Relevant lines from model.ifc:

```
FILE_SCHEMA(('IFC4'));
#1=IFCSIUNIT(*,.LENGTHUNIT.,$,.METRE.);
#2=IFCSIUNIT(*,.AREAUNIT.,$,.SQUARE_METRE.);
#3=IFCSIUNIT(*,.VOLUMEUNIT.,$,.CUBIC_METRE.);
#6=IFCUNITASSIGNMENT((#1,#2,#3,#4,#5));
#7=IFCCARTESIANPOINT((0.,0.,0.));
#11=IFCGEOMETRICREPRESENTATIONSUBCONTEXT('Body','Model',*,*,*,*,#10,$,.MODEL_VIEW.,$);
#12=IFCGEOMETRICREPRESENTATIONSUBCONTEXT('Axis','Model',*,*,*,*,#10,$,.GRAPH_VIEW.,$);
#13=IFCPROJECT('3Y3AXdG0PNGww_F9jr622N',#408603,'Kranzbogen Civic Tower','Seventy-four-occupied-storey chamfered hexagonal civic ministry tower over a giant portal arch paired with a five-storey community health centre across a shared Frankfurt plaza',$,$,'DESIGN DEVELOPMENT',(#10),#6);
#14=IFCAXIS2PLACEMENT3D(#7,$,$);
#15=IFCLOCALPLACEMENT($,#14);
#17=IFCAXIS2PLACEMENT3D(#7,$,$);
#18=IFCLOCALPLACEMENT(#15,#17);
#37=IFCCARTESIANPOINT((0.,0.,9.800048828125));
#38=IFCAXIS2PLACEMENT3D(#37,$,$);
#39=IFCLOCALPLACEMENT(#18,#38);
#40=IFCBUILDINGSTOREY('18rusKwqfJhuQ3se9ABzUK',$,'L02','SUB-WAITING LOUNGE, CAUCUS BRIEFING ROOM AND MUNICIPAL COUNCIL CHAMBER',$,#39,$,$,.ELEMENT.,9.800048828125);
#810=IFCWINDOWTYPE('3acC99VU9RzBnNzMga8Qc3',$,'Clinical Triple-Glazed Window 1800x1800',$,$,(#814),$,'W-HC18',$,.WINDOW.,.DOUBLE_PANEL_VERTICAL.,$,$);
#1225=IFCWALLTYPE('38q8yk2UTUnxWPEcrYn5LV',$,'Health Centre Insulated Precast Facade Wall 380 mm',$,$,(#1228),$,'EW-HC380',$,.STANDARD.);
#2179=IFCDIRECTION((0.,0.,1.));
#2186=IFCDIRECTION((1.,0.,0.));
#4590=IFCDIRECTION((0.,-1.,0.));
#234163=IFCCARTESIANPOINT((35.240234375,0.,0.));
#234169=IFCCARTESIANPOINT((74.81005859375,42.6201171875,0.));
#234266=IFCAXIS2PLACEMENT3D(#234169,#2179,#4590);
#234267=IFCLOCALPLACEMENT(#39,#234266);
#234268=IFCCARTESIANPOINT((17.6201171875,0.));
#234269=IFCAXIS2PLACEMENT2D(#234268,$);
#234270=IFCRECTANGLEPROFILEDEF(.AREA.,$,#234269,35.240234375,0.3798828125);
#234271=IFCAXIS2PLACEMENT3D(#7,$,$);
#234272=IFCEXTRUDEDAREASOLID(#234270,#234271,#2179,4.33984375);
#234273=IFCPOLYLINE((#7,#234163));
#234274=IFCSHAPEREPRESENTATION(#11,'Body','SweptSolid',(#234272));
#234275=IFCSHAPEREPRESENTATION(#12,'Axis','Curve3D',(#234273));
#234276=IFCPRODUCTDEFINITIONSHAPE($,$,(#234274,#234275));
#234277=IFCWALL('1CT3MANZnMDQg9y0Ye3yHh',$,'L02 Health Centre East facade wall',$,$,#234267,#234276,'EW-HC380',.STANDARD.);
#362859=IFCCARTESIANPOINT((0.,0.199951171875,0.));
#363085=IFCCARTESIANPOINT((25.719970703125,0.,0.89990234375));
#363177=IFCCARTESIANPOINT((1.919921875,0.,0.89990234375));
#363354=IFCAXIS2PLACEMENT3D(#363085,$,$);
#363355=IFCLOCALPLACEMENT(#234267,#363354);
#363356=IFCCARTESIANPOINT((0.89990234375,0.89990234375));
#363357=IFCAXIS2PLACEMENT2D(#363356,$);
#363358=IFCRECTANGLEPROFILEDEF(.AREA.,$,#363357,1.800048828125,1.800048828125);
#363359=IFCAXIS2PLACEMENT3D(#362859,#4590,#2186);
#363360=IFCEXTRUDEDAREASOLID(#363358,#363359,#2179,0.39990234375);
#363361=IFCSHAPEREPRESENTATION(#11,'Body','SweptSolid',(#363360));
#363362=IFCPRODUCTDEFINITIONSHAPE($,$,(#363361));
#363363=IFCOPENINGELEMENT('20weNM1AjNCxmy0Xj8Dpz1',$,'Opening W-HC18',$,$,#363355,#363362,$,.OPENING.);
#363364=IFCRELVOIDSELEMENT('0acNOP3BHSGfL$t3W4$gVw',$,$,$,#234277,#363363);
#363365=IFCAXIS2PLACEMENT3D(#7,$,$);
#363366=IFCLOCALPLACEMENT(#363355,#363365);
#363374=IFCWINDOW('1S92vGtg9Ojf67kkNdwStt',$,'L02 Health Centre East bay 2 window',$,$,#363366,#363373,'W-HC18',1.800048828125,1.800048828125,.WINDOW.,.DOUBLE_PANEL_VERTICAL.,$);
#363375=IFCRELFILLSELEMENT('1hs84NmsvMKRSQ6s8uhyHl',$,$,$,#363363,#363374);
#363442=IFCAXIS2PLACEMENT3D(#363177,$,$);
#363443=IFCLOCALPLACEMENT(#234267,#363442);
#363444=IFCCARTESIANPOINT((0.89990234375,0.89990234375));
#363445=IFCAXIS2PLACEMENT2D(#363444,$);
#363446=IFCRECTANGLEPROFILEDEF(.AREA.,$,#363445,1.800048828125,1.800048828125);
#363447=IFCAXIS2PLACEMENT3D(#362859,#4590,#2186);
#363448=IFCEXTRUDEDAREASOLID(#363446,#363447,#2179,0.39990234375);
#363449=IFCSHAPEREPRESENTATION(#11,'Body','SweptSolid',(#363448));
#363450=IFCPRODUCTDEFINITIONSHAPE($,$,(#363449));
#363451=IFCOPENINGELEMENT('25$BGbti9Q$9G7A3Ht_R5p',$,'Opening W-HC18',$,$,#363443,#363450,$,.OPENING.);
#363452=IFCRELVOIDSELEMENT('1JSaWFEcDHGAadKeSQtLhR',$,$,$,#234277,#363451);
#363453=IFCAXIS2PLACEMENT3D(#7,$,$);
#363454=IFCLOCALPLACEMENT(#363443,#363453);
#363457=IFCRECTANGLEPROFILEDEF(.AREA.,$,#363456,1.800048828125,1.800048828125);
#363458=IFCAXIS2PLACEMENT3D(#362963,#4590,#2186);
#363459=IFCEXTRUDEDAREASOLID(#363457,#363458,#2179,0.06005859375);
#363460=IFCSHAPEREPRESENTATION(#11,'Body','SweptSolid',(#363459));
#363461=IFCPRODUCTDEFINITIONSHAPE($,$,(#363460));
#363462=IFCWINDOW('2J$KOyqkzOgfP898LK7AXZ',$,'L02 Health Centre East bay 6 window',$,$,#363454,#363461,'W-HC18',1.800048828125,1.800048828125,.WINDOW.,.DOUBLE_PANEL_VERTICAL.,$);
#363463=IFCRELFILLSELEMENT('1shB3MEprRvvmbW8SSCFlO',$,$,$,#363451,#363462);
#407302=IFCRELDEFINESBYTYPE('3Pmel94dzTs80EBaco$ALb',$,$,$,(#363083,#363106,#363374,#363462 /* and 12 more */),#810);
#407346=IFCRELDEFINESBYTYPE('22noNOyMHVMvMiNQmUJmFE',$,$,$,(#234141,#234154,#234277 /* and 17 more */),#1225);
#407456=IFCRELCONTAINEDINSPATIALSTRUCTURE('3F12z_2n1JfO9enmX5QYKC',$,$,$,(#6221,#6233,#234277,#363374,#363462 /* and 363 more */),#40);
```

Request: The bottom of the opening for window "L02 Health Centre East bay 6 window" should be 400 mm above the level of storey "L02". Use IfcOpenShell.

```python
import numpy as np
import ifcopenshell
import ifcopenshell.api.geometry
import ifcopenshell.geom
import ifcopenshell.util.element
import ifcopenshell.util.placement
import ifcopenshell.util.shape
import ifcopenshell.util.unit

model = ifcopenshell.open("model.ifc")
unit_scale = ifcopenshell.util.unit.calculate_unit_scale(model)

window = model.by_id(363462)
opening = window.FillsVoids[0].RelatingOpeningElement
storey = ifcopenshell.util.element.get_container(window, ifc_class="IfcBuildingStorey")
level = ifcopenshell.util.placement.get_local_placement(storey.ObjectPlacement)[2, 3]

# The opening's origin need not be at the sill, so measure its lowest point.
shape = ifcopenshell.geom.create_shape(ifcopenshell.geom.settings(), opening)
bottom = ifcopenshell.util.shape.get_shape_bottom_elevation(shape, shape.geometry) / unit_scale
dz = level + 0.4 - bottom

shift = np.array([0.0, 0.0, dz])
# The window is placed relative to its opening, so it follows when the opening moves.
matrix = ifcopenshell.util.placement.get_local_placement(opening.ObjectPlacement)
matrix[:3, 3] += shift
ifcopenshell.api.geometry.edit_object_placement(
    model, product=opening, matrix=matrix, is_si=False, should_transform_children=True
)

print(f"moved by {dz * unit_scale:+.3f} m")

model.write("model_rev.ifc")
```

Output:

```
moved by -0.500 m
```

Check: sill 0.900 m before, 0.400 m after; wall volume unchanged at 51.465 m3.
